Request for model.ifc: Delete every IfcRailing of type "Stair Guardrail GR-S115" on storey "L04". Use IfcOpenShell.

First a look at what the model holds.

```python
import ifcopenshell
import ifcopenshell.util.element

model = ifcopenshell.open("model.ifc")
print(model.schema)
storey = next(s for s in model.by_type("IfcBuildingStorey") if s.Name == "L04")
railings = [e for e in ifcopenshell.util.element.get_decomposition(storey) if e.is_a("IfcRailing")]
seen = {}
for e in railings:
    element_type = ifcopenshell.util.element.get_type(e)
    name = element_type.Name if element_type not in (None, e) else None
    seen[name] = seen.get(name, 0) + 1
for name, count in sorted(seen.items(), key=str):
    print(count, "x", name)
```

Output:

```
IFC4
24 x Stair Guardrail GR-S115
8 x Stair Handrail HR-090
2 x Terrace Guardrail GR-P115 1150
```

```python
import ifcopenshell
import ifcopenshell.api.root
import ifcopenshell.util.element

model = ifcopenshell.open("model.ifc")

storey = next(s for s in model.by_type("IfcBuildingStorey") if s.Name == "L04")
railings = [e for e in ifcopenshell.util.element.get_decomposition(storey) if e.is_a("IfcRailing")]
targets = [e for e in railings if (t := ifcopenshell.util.element.get_type(e)) not in (None, e) and t.Name == "Stair Guardrail GR-S115"]

for e in targets:
    ifcopenshell.api.root.remove_product(model, product=e)
print(len(targets), "removed")

model.write("model_edited.ifc")
```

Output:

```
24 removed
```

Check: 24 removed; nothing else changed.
